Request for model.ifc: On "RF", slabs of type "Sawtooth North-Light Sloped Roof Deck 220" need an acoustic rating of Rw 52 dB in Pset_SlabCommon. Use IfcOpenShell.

First a look at what the model holds.

```python
import ifcopenshell
import ifcopenshell.util.element

model = ifcopenshell.open("model.ifc")
print(model.schema)
storey = next(s for s in model.by_type("IfcBuildingStorey") if s.Name == "RF")
slabs = [e for e in ifcopenshell.util.element.get_decomposition(storey) if e.is_a("IfcSlab")]
seen = {}
for e in slabs:
    element_type = ifcopenshell.util.element.get_type(e)
    key = (element_type.Name if element_type != e and element_type else None, ifcopenshell.util.element.get_pset(e, "Pset_SlabCommon", "AcousticRating"))
    seen[key] = seen.get(key, 0) + 1
for (name, value), count in sorted(seen.items(), key=str):
    print(count, "x", name, "|", value)
```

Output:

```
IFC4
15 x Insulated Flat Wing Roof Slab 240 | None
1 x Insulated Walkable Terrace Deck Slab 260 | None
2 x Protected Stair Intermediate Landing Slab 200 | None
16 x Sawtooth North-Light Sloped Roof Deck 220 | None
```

```python
import ifcopenshell
import ifcopenshell.api.pset
import ifcopenshell.util.element

model = ifcopenshell.open("model.ifc")

storey = next(s for s in model.by_type("IfcBuildingStorey") if s.Name == "RF")
slabs = [e for e in ifcopenshell.util.element.get_decomposition(storey) if e.is_a("IfcSlab")]

count = 0
for e in slabs:
    element_type = ifcopenshell.util.element.get_type(e)
    if element_type in (None, e) or element_type.Name != "Sawtooth North-Light Sloped Roof Deck 220":
        continue
    # add_pset returns the element's existing set when there is one.
    pset = ifcopenshell.api.pset.add_pset(model, product=e, name="Pset_SlabCommon")
    ifcopenshell.api.pset.edit_pset(model, pset=pset, properties={"AcousticRating": "Rw 52 dB"})
    count += 1

print(count, "slabs updated")

model.write("model_edited.ifc")
```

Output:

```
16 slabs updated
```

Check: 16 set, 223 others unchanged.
